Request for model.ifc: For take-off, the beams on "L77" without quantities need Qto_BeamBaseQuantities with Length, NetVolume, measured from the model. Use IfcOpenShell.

First a look at what the model holds.

```python
import ifcopenshell
import ifcopenshell.util.element
import ifcopenshell.util.unit

model = ifcopenshell.open("model.ifc")
print(model.schema)
for unit_type in ("LENGTHUNIT", "AREAUNIT", "VOLUMEUNIT"):
    print(unit_type, ifcopenshell.util.unit.calculate_unit_scale(model, unit_type))
storey = next(s for s in model.by_type("IfcBuildingStorey") if s.Name == "L77")
beams = [e for e in ifcopenshell.util.element.get_decomposition(storey) if e.is_a("IfcBeam")]
for e in sorted(beams, key=lambda e: e.id()):
    print(e.id(), e.is_a(), e.Name, list(ifcopenshell.util.element.get_psets(e, qtos_only=True)), sep=" | ")
```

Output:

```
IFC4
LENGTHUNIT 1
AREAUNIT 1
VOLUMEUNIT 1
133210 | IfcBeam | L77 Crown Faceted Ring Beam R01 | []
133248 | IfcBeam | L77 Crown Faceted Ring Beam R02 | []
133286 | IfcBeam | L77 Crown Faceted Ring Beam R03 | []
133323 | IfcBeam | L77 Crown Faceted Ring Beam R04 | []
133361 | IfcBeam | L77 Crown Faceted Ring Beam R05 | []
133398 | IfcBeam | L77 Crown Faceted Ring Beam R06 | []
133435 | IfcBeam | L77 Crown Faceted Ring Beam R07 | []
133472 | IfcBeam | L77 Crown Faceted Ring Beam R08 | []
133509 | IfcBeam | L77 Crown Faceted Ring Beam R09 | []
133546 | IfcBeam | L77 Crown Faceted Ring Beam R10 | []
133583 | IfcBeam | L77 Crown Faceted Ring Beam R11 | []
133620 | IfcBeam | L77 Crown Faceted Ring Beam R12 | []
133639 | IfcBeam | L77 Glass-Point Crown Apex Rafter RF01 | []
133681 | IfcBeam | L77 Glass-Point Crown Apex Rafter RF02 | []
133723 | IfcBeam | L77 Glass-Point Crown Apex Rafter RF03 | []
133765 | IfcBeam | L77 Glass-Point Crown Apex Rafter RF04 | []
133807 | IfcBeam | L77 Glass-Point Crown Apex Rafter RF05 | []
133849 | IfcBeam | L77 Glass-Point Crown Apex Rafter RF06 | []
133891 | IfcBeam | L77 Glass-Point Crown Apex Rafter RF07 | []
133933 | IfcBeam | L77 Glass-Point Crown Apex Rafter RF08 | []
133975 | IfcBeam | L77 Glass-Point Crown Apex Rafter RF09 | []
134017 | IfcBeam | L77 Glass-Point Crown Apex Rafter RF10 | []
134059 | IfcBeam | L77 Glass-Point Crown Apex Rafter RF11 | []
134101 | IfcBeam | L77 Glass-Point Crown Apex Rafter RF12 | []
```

```python
import ifcopenshell
import ifcopenshell.api.pset
import ifcopenshell.geom
import ifcopenshell.util.element
import ifcopenshell.util.shape
import ifcopenshell.util.unit

model = ifcopenshell.open("model.ifc")
unit_scale = ifcopenshell.util.unit.calculate_unit_scale(model)
volume_scale = ifcopenshell.util.unit.calculate_unit_scale(model, "VOLUMEUNIT")
settings = ifcopenshell.geom.settings()

storey = next(s for s in model.by_type("IfcBuildingStorey") if s.Name == "L77")
beams = [e for e in ifcopenshell.util.element.get_decomposition(storey) if e.is_a("IfcBeam")]

for e in sorted(beams, key=lambda e: e.id()):
    if ifcopenshell.util.element.get_psets(e, qtos_only=True, should_inherit=False):
        continue
    # Geometry comes back in metres, in the element's own axes.
    shape = ifcopenshell.geom.create_shape(settings, e)
    values = {
        "Length": ifcopenshell.util.shape.get_max_xyz(shape.geometry) / unit_scale,
        "NetVolume": ifcopenshell.util.shape.get_volume(shape.geometry) / volume_scale,
    }
    qto = ifcopenshell.api.pset.add_qto(model, product=e, name="Qto_BeamBaseQuantities")
    ifcopenshell.api.pset.edit_qto(model, qto=qto, properties=values)
    print(e.id(), {k: round(v, 3) for k, v in values.items()})

model.write("model_v2.ifc")
```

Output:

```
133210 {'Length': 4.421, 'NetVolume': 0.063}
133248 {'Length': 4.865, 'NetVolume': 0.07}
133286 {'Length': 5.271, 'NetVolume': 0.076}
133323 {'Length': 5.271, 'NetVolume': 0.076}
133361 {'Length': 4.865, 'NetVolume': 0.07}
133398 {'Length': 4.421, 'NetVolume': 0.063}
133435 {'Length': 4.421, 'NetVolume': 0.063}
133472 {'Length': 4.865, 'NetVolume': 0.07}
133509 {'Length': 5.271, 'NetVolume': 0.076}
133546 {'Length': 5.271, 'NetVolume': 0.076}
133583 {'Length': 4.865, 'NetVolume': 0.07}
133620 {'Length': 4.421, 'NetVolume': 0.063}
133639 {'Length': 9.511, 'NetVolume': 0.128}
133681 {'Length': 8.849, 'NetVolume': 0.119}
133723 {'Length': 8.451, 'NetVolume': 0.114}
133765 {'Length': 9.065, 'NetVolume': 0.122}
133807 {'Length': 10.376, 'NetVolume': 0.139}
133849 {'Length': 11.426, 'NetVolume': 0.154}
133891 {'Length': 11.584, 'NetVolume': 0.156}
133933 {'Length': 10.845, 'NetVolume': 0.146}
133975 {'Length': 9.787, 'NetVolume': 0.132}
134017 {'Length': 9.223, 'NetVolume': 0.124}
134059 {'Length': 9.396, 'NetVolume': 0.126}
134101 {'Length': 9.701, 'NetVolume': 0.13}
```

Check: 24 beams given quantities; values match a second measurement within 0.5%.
